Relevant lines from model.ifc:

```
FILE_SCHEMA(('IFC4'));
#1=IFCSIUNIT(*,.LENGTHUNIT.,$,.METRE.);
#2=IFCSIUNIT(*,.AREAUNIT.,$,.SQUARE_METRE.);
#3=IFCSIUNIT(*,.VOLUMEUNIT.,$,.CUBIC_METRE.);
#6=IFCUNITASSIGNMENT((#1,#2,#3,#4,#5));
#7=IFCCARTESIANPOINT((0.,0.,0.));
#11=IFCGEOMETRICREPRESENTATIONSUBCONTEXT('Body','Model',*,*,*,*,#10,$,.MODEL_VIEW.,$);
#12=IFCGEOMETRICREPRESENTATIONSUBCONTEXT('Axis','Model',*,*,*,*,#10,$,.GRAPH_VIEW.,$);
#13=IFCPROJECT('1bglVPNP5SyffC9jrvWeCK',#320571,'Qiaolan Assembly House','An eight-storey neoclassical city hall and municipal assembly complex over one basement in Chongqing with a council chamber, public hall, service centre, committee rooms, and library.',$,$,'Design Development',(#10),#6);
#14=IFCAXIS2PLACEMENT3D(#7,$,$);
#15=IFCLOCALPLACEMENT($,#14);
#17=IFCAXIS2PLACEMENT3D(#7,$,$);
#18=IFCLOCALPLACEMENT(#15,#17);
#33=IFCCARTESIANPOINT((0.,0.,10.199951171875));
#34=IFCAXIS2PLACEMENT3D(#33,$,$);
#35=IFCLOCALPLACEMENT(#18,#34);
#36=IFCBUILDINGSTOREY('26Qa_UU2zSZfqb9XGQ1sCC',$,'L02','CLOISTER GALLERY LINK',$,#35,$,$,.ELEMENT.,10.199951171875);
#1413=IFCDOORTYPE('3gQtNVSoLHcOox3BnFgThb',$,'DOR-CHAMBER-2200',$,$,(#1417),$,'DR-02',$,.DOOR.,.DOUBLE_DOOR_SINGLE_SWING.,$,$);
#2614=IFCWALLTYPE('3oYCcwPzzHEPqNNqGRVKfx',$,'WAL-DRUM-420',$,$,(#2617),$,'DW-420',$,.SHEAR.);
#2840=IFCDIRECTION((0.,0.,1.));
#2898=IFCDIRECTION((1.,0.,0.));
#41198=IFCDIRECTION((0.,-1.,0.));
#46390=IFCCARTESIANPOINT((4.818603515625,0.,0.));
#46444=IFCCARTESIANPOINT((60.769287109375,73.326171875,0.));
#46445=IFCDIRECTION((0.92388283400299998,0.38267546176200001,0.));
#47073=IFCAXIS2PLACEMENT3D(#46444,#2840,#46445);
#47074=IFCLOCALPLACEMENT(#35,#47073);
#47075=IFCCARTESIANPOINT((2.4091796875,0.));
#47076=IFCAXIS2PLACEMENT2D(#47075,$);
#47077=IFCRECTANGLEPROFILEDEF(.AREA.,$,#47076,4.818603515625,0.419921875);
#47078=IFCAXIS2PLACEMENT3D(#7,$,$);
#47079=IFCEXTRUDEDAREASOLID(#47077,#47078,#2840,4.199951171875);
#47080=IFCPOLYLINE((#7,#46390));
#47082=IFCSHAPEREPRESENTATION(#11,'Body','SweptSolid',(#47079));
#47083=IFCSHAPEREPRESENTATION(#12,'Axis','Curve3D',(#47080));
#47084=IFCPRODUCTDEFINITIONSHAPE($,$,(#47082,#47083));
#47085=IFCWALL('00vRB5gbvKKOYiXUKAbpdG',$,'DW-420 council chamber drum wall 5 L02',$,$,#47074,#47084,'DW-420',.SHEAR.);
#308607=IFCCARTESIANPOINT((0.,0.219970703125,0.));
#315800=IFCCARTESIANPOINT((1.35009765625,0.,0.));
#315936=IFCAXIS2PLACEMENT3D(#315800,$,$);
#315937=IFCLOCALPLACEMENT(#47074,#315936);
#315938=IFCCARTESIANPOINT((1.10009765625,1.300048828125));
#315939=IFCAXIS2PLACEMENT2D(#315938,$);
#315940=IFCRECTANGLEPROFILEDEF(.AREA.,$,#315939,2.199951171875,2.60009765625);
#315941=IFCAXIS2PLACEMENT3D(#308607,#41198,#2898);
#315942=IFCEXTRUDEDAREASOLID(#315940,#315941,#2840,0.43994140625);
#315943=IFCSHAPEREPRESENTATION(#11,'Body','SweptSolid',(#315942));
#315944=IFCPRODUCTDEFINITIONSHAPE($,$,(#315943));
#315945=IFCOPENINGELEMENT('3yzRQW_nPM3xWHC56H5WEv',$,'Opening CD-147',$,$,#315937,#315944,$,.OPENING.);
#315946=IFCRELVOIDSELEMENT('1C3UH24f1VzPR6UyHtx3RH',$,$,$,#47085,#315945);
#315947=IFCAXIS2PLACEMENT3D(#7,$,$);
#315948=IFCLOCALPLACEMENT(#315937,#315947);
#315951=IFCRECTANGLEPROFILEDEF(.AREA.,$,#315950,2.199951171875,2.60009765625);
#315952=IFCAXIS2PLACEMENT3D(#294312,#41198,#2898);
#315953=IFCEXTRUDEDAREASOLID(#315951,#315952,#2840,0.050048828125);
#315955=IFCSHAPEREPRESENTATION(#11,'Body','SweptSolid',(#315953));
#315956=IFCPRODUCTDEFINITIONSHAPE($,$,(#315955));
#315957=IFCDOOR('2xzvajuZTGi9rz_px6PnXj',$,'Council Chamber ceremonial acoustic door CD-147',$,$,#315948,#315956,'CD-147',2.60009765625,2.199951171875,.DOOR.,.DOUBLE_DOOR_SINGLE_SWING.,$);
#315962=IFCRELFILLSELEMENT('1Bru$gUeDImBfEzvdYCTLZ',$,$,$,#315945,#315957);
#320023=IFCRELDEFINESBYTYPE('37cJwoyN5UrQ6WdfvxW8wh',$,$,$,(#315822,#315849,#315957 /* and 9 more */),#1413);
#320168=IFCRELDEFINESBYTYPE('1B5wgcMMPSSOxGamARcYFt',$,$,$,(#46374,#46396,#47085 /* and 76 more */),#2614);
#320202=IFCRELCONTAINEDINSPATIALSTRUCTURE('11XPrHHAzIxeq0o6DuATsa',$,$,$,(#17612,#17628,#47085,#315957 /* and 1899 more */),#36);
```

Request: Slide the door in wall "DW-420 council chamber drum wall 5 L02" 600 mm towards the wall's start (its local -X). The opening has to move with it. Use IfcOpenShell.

```python
import ifcopenshell
import ifcopenshell.api.geometry
import ifcopenshell.util.placement
import ifcopenshell.util.unit

model = ifcopenshell.open("model.ifc")
unit_scale = ifcopenshell.util.unit.calculate_unit_scale(model)

door = model.by_guid("2xzvajuZTGi9rz_px6PnXj")
opening = door.FillsVoids[0].RelatingOpeningElement
wall = opening.VoidsElements[0].RelatingBuildingElement

wall_matrix = ifcopenshell.util.placement.get_local_placement(wall.ObjectPlacement)
shift = wall_matrix[:3, 0] * -0.6 / unit_scale
before = ifcopenshell.util.placement.get_local_placement(door.ObjectPlacement)[:3, 3].copy()

# The door is placed relative to its opening, so it follows when the opening moves.
matrix = ifcopenshell.util.placement.get_local_placement(opening.ObjectPlacement)
matrix[:3, 3] += shift
ifcopenshell.api.geometry.edit_object_placement(
    model, product=opening, matrix=matrix, is_si=False, should_transform_children=True
)

after = ifcopenshell.util.placement.get_local_placement(door.ObjectPlacement)[:3, 3]
print("door moved by", (after - before).round(3) + 0.0)

model.write("model_rev.ifc")
```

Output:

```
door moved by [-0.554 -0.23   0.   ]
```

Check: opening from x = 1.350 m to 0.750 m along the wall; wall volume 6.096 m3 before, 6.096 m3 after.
